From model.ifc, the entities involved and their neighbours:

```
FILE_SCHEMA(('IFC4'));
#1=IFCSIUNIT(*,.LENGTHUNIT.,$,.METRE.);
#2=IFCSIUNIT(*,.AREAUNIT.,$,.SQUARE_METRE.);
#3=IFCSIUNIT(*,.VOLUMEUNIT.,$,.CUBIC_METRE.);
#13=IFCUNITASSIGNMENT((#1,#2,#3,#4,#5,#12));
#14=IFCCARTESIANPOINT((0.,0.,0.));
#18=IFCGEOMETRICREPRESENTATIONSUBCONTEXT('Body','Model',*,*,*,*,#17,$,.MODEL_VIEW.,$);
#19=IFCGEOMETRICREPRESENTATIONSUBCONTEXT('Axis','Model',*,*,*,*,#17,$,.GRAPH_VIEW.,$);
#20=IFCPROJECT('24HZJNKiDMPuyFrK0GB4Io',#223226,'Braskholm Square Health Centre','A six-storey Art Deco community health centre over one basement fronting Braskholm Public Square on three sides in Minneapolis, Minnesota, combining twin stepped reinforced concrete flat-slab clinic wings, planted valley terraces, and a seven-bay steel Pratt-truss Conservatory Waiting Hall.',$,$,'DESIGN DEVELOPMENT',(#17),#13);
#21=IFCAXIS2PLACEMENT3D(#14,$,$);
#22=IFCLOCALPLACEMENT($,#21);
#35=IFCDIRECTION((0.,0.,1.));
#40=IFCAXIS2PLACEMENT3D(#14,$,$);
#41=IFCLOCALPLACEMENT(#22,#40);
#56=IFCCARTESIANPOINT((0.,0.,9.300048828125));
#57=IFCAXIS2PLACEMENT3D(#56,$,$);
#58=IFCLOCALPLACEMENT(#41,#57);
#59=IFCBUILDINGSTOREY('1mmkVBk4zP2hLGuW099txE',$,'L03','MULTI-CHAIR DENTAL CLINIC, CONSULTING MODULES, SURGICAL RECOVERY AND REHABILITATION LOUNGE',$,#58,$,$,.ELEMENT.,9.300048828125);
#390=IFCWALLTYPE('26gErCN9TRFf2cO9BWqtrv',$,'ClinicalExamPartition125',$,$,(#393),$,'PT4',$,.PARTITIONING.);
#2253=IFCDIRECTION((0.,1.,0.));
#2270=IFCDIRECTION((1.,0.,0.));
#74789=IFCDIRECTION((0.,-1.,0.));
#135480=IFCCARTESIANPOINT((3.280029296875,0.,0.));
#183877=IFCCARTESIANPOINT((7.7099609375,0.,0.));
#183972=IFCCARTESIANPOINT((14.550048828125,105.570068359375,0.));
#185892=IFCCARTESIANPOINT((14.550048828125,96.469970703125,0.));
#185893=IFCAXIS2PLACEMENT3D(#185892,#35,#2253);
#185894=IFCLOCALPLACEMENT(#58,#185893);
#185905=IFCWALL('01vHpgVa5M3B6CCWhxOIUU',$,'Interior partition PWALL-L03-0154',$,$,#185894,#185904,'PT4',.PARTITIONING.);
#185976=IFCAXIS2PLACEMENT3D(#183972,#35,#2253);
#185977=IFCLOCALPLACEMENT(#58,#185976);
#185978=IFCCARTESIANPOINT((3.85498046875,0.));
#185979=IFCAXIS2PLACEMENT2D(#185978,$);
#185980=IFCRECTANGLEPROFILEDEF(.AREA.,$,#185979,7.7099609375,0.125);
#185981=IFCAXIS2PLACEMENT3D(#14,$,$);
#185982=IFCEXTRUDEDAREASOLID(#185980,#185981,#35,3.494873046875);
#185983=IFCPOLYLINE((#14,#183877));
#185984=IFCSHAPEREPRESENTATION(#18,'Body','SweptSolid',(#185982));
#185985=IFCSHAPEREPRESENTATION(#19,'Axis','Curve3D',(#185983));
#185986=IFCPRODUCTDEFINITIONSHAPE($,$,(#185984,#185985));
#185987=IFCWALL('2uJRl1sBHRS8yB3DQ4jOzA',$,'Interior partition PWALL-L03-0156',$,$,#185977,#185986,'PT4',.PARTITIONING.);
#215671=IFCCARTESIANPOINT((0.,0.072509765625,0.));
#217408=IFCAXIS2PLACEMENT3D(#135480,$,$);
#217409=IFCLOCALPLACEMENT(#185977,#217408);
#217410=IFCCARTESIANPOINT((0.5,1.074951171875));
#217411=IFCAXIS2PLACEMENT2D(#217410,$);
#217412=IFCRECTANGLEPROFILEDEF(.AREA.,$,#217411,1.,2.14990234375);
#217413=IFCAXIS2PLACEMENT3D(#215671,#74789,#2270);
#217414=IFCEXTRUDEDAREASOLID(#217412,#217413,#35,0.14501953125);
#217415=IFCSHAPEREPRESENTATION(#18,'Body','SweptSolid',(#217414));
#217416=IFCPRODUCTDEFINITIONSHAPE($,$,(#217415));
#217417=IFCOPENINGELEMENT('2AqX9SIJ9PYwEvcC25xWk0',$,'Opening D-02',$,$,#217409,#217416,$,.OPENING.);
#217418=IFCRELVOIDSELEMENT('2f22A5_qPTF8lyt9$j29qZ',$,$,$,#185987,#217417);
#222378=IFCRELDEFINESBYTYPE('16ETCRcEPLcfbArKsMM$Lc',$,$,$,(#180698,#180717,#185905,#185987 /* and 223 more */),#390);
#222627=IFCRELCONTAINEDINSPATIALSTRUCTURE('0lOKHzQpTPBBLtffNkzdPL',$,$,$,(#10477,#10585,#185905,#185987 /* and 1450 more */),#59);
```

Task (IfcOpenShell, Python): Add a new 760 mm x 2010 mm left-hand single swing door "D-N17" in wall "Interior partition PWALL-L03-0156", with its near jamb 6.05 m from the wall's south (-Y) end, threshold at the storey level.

```python
import numpy as np
import ifcopenshell
import ifcopenshell.api.feature
import ifcopenshell.api.geometry
import ifcopenshell.api.root
import ifcopenshell.api.spatial
import ifcopenshell.geom
import ifcopenshell.util.element
import ifcopenshell.util.placement
import ifcopenshell.util.representation
import ifcopenshell.util.shape
import ifcopenshell.util.unit

model = ifcopenshell.open("model.ifc")
unit_scale = ifcopenshell.util.unit.calculate_unit_scale(model)
settings = ifcopenshell.geom.settings()


def volume(element):
    """Net volume in cubic metres, openings subtracted."""
    shape = ifcopenshell.geom.create_shape(settings, element)
    return ifcopenshell.util.shape.get_volume(shape.geometry)


wall = model.by_guid("2uJRl1sBHRS8yB3DQ4jOzA")
storey = ifcopenshell.util.element.get_container(wall, ifc_class="IfcBuildingStorey")
context = ifcopenshell.util.representation.get_context(model, "Model", "Body", "MODEL_VIEW")
before = volume(wall)

width, height, from_end, sill = 0.76, 2.01, 6.05, 0.0  # metres

# The wall runs along its own X axis, and the end named is its -X end.
wall_shape = ifcopenshell.geom.create_shape(settings, wall)
x, y, z = ifcopenshell.util.shape.get_vertices(wall_shape.geometry).T
start = x.min() + from_end
face, thickness = float(y.min()), float(y.max() - y.min())
wall_matrix = ifcopenshell.util.placement.get_local_placement(wall.ObjectPlacement)
level = ifcopenshell.util.placement.get_local_placement(storey.ObjectPlacement)[2, 3]


def in_wall(x, y):
    """Placement at x, y metres in the wall's axes, at sill height."""
    matrix = wall_matrix.copy()
    matrix[:, 3] = wall_matrix @ np.array([x / unit_scale, y / unit_scale, 0.0, 1.0])
    matrix[2, 3] = level + sill / unit_scale
    return matrix


# Opening: a box that overshoots both wall faces by 50 mm.
opening = ifcopenshell.api.root.create_entity(model, ifc_class="IfcOpeningElement", predefined_type="OPENING")
box = ifcopenshell.api.geometry.add_wall_representation(
    model, context=context, length=width, height=height, thickness=thickness + 0.1
)
ifcopenshell.api.geometry.assign_representation(model, product=opening, representation=box)
ifcopenshell.api.geometry.edit_object_placement(model, product=opening, matrix=in_wall(start, face - 0.05), is_si=False)
ifcopenshell.api.feature.add_feature(model, feature=opening, element=wall)

door = ifcopenshell.api.root.create_entity(model, ifc_class="IfcDoor", name="D-N17", predefined_type="DOOR")
door.OverallWidth, door.OverallHeight = width / unit_scale, height / unit_scale
door.OperationType = "SINGLE_SWING_LEFT"
body = ifcopenshell.api.geometry.add_door_representation(
    model,
    context=context,
    overall_width=door.OverallWidth,
    overall_height=door.OverallHeight,
    operation_type="SINGLE_SWING_LEFT",
    lining_properties={"LiningDepth": thickness / unit_scale, "ThresholdDepth": thickness / unit_scale},
)
ifcopenshell.api.geometry.assign_representation(model, product=door, representation=body)
ifcopenshell.api.spatial.assign_container(model, products=[door], relating_structure=storey)
ifcopenshell.api.feature.add_filling(model, opening=opening, element=door)

# The lining spans the wall, so the door starts at the wall face.
ifcopenshell.api.geometry.edit_object_placement(model, product=door, matrix=in_wall(start, face), is_si=False)

after = volume(wall)

print(f"wall volume {before:.3f} -> {after:.3f} m3")

model.write("model-out.ifc")
```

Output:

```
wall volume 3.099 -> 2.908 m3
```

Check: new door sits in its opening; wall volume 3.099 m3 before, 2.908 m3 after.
